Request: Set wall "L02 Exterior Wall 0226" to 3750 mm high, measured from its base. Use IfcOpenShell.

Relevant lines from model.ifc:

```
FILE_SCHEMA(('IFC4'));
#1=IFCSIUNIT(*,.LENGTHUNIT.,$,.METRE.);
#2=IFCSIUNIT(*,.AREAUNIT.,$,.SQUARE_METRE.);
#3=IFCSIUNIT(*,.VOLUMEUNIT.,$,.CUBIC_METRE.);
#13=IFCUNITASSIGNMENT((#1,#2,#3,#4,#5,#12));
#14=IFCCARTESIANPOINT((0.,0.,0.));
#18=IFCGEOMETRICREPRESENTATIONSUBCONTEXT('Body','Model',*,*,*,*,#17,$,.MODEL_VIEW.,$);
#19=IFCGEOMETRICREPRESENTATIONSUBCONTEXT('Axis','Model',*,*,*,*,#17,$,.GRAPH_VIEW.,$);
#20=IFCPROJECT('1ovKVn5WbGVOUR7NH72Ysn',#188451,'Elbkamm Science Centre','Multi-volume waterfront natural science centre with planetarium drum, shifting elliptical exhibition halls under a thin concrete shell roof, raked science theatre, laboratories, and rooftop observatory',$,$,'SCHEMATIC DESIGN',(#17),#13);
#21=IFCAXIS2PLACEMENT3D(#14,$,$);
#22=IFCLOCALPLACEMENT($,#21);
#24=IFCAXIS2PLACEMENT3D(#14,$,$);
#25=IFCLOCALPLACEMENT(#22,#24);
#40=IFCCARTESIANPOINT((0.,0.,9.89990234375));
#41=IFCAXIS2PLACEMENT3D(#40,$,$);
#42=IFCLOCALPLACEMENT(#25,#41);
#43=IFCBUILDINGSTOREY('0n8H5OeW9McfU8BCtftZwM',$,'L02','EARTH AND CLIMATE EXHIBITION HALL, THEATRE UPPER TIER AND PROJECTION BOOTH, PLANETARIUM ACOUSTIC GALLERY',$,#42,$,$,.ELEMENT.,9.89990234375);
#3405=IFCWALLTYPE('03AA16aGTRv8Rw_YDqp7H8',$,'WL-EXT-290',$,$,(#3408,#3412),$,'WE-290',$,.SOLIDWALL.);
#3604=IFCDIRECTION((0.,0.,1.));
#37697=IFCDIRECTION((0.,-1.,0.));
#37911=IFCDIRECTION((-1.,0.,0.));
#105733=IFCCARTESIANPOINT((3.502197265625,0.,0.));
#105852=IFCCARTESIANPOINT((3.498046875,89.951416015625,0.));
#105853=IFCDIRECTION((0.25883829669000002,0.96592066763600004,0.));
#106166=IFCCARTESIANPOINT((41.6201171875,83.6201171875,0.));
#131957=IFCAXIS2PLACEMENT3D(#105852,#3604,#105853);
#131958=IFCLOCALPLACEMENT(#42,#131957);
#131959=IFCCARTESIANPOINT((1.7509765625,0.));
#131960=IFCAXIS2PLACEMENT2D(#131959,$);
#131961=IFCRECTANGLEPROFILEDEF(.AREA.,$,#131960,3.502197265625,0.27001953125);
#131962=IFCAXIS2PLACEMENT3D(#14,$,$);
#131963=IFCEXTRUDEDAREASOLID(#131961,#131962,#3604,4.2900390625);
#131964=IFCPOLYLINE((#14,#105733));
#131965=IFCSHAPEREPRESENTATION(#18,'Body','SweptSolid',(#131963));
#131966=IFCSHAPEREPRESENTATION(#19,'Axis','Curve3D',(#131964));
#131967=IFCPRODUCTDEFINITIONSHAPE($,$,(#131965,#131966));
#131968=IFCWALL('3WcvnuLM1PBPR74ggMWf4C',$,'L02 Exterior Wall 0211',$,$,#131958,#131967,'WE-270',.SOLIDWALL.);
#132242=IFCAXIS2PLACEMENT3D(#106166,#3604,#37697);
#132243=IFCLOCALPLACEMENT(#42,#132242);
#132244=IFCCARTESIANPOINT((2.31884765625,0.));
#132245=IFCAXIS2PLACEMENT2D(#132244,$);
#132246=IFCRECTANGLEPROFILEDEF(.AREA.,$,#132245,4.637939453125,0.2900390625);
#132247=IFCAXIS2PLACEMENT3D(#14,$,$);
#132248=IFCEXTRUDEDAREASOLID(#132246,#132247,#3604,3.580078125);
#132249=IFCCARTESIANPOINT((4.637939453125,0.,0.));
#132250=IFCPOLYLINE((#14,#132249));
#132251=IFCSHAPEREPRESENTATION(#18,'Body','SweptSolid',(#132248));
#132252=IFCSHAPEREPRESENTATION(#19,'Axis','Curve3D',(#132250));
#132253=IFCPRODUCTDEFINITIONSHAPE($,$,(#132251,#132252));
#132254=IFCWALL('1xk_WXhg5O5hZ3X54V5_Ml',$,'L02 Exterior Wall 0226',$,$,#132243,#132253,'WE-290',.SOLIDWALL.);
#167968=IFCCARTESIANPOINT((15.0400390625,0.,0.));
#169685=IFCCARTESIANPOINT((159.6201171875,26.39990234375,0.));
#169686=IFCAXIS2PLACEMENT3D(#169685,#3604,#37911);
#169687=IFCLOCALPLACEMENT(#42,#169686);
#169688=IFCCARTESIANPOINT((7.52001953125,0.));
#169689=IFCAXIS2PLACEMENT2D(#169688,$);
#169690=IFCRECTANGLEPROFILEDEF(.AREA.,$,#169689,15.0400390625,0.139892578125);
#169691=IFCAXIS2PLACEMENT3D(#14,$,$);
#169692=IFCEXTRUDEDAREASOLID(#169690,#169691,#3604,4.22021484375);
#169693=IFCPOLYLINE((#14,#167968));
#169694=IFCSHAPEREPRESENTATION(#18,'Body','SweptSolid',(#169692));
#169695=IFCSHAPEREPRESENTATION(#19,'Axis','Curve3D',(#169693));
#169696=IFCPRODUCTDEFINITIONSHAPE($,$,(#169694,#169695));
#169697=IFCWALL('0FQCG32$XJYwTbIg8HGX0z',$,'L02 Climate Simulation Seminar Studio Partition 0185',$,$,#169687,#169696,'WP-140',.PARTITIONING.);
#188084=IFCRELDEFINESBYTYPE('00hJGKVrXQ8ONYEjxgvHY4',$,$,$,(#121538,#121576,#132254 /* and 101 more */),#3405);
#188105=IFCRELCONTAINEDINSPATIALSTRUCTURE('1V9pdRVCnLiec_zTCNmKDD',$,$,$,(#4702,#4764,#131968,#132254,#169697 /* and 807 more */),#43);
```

```python
import ifcopenshell
import ifcopenshell.geom
import ifcopenshell.util.representation
import ifcopenshell.util.shape

model = ifcopenshell.open("model.ifc")
settings = ifcopenshell.geom.settings()


def volume(element):
    """Net volume in cubic metres, openings subtracted."""
    shape = ifcopenshell.geom.create_shape(settings, element)
    return ifcopenshell.util.shape.get_volume(shape.geometry)


wall = model.by_guid("1xk_WXhg5O5hZ3X54V5_Ml")
before = volume(wall)

body = ifcopenshell.util.representation.get_representation(wall, "Model", "Body")
solid = body.Items[0]
old_height = solid.Depth
solid.Depth = 3.75
after = volume(wall)

print(f"height {old_height:g} -> {solid.Depth:g}, volume {before:.3f} -> {after:.3f} m3")

model.write("model_v2.ifc")
```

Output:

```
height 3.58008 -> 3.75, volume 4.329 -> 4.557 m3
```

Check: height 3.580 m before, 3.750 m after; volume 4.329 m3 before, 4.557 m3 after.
